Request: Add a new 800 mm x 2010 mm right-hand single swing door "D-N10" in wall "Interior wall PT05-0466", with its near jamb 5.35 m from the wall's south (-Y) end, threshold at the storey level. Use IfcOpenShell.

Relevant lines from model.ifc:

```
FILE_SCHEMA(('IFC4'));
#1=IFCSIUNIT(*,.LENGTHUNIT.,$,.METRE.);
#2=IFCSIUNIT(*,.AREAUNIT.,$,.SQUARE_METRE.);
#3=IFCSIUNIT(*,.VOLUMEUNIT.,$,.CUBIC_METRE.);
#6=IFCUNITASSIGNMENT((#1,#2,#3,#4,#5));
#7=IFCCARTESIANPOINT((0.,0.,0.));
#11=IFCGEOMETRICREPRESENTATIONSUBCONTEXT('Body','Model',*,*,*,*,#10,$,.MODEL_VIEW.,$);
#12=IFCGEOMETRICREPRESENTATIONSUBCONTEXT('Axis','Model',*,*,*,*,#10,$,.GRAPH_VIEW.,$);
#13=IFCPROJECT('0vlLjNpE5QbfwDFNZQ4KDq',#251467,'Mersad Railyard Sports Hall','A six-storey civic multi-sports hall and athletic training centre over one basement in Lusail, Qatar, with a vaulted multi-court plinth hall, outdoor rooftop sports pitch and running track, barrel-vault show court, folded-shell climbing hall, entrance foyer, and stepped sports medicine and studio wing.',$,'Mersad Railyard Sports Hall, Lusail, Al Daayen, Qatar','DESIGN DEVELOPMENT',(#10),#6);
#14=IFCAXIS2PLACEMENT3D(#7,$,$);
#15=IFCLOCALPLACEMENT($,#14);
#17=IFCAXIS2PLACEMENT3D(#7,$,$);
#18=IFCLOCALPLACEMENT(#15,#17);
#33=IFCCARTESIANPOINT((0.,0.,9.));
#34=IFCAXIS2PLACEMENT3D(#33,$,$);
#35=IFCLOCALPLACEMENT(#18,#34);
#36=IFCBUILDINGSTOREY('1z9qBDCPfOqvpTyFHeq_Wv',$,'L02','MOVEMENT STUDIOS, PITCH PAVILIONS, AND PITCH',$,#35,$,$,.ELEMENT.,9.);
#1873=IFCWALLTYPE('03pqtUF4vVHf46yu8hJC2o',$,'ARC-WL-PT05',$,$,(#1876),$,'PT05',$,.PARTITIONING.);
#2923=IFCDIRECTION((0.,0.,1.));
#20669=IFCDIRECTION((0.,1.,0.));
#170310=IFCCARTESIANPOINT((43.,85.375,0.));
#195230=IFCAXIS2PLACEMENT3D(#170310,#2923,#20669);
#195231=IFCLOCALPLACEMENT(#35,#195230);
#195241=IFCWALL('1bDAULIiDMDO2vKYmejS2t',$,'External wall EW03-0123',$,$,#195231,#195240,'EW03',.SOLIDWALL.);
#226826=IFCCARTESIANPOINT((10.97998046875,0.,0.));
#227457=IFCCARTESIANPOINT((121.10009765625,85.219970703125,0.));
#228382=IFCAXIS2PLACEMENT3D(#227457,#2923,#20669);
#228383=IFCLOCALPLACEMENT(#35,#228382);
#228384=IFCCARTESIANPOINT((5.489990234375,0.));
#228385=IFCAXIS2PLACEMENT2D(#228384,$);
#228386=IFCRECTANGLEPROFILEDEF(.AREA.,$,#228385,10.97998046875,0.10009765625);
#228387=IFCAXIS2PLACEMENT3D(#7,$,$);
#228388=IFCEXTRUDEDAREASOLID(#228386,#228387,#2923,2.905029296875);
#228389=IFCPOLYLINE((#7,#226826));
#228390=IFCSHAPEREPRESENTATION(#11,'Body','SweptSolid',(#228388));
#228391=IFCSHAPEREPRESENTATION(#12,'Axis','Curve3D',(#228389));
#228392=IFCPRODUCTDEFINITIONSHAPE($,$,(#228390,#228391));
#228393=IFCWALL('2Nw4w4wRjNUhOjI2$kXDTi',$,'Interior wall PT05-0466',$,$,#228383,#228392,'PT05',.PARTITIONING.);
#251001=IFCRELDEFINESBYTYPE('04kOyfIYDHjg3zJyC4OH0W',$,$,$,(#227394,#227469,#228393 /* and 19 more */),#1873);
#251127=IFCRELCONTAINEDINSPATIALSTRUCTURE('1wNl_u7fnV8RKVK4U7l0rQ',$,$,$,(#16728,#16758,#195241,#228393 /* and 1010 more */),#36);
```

```python
import numpy as np
import ifcopenshell
import ifcopenshell.api.feature
import ifcopenshell.api.geometry
import ifcopenshell.api.root
import ifcopenshell.api.spatial
import ifcopenshell.geom
import ifcopenshell.util.element
import ifcopenshell.util.placement
import ifcopenshell.util.representation
import ifcopenshell.util.shape
import ifcopenshell.util.unit

model = ifcopenshell.open("model.ifc")
unit_scale = ifcopenshell.util.unit.calculate_unit_scale(model)
settings = ifcopenshell.geom.settings()


def volume(element):
    """Net volume in cubic metres, openings subtracted."""
    shape = ifcopenshell.geom.create_shape(settings, element)
    return ifcopenshell.util.shape.get_volume(shape.geometry)


wall = model.by_guid("2Nw4w4wRjNUhOjI2$kXDTi")
storey = ifcopenshell.util.element.get_container(wall, ifc_class="IfcBuildingStorey")
context = ifcopenshell.util.representation.get_context(model, "Model", "Body", "MODEL_VIEW")
before = volume(wall)

width, height, from_end, sill = 0.8, 2.01, 5.35, 0.0  # metres

# The wall runs along its own X axis, and the end named is its -X end.
wall_shape = ifcopenshell.geom.create_shape(settings, wall)
x, y, z = ifcopenshell.util.shape.get_vertices(wall_shape.geometry).T
start = x.min() + from_end
face, thickness = float(y.min()), float(y.max() - y.min())
wall_matrix = ifcopenshell.util.placement.get_local_placement(wall.ObjectPlacement)
level = ifcopenshell.util.placement.get_local_placement(storey.ObjectPlacement)[2, 3]


def in_wall(x, y):
    """Placement at x, y metres in the wall's axes, at sill height."""
    matrix = wall_matrix.copy()
    matrix[:, 3] = wall_matrix @ np.array([x / unit_scale, y / unit_scale, 0.0, 1.0])
    matrix[2, 3] = level + sill / unit_scale
    return matrix


# Opening: a box that overshoots both wall faces by 50 mm.
opening = ifcopenshell.api.root.create_entity(model, ifc_class="IfcOpeningElement", predefined_type="OPENING")
box = ifcopenshell.api.geometry.add_wall_representation(
    model, context=context, length=width, height=height, thickness=thickness + 0.1
)
ifcopenshell.api.geometry.assign_representation(model, product=opening, representation=box)
ifcopenshell.api.geometry.edit_object_placement(model, product=opening, matrix=in_wall(start, face - 0.05), is_si=False)
ifcopenshell.api.feature.add_feature(model, feature=opening, element=wall)

door = ifcopenshell.api.root.create_entity(model, ifc_class="IfcDoor", name="D-N10", predefined_type="DOOR")
door.OverallWidth, door.OverallHeight = width / unit_scale, height / unit_scale
door.OperationType = "SINGLE_SWING_RIGHT"
body = ifcopenshell.api.geometry.add_door_representation(
    model,
    context=context,
    overall_width=door.OverallWidth,
    overall_height=door.OverallHeight,
    operation_type="SINGLE_SWING_RIGHT",
    lining_properties={"LiningDepth": thickness / unit_scale, "ThresholdDepth": thickness / unit_scale},
)
ifcopenshell.api.geometry.assign_representation(model, product=door, representation=body)
ifcopenshell.api.spatial.assign_container(model, products=[door], relating_structure=storey)
ifcopenshell.api.feature.add_filling(model, opening=opening, element=door)

# The lining spans the wall, so the door starts at the wall face.
ifcopenshell.api.geometry.edit_object_placement(model, product=door, matrix=in_wall(start, face), is_si=False)

after = volume(wall)

print(f"wall volume {before:.3f} -> {after:.3f} m3")

model.write("model_updated.ifc")
```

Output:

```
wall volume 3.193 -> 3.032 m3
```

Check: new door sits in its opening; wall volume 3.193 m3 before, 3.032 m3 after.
